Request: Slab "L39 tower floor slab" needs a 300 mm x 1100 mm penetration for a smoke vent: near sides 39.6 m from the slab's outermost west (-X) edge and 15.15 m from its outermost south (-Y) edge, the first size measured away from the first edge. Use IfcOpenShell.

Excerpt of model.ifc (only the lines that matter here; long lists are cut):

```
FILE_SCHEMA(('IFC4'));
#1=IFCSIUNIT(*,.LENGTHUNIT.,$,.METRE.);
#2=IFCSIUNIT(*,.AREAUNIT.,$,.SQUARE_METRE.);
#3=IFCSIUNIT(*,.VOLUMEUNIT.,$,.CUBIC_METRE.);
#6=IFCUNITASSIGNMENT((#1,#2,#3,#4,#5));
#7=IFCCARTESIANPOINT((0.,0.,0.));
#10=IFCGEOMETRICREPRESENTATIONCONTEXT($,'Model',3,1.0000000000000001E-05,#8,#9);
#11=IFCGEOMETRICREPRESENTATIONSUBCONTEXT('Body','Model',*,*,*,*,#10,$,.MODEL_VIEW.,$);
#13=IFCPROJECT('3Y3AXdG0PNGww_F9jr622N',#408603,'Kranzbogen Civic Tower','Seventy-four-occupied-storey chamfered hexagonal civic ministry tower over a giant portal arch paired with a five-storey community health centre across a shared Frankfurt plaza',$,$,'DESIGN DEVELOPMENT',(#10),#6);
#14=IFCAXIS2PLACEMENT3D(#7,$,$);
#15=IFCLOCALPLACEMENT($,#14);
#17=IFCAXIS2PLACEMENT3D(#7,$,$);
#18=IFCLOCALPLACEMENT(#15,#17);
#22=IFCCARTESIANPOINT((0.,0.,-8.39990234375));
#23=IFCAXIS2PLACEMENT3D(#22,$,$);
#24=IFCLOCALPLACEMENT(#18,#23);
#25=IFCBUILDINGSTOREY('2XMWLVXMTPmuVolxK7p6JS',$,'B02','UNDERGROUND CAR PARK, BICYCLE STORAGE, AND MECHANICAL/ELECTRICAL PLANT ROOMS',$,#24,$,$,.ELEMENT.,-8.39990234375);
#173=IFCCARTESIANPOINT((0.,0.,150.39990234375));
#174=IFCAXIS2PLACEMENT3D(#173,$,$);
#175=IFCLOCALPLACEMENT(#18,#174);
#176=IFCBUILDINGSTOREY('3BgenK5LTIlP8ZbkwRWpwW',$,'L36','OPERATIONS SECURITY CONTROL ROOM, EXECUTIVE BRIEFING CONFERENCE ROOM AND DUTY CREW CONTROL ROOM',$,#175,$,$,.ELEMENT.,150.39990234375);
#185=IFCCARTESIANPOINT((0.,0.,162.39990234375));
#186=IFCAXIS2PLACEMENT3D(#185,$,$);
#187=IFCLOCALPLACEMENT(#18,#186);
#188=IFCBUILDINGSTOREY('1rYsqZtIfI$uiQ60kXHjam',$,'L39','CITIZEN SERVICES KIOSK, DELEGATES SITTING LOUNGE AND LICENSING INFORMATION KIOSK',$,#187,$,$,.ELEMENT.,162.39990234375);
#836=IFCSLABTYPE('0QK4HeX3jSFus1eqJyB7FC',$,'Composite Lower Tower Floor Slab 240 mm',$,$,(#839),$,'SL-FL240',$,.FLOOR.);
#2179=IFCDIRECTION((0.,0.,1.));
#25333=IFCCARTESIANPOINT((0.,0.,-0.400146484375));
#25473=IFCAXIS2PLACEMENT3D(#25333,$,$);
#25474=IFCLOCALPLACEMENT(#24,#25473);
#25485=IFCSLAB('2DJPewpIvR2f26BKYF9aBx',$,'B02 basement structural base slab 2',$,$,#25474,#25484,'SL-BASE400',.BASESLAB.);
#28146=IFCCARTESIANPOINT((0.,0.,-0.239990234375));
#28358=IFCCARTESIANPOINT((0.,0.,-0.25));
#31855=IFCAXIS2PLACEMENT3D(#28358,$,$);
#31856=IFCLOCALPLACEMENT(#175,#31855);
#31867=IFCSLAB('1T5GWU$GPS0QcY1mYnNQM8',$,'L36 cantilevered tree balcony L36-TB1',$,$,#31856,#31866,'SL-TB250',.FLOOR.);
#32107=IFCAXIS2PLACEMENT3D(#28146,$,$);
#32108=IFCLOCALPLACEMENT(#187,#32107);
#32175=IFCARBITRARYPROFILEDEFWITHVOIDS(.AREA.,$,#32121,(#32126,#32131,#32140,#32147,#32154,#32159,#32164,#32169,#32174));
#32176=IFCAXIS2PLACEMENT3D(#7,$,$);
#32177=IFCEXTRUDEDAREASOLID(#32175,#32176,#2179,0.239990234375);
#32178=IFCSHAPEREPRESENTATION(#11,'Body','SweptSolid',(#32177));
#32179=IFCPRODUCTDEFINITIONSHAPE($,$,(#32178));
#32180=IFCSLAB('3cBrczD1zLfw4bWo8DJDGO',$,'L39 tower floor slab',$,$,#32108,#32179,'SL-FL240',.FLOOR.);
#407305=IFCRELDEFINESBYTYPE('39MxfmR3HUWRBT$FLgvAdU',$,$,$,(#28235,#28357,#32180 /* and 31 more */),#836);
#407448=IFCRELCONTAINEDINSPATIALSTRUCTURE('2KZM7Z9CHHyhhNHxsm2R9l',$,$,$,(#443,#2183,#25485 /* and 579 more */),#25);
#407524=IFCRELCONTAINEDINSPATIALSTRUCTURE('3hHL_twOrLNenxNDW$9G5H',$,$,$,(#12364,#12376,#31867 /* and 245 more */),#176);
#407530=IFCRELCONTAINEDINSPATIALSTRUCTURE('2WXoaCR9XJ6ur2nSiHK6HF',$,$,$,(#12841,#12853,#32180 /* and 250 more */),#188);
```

```python
import numpy as np
import ifcopenshell
import ifcopenshell.api.feature
import ifcopenshell.api.geometry
import ifcopenshell.api.root
import ifcopenshell.geom
import ifcopenshell.util.placement
import ifcopenshell.util.representation
import ifcopenshell.util.shape
import ifcopenshell.util.unit

model = ifcopenshell.open("model.ifc")
unit_scale = ifcopenshell.util.unit.calculate_unit_scale(model)
settings = ifcopenshell.geom.settings()


def volume(element):
    """Net volume in cubic metres, openings subtracted."""
    shape = ifcopenshell.geom.create_shape(settings, element)
    return ifcopenshell.util.shape.get_volume(shape.geometry)


slab = model.by_id(32180)
before = volume(slab)

# Extent in the slab's own axes, in metres. The edges named are its -X and -Y sides.
slab_shape = ifcopenshell.geom.create_shape(settings, slab)
vertices = ifcopenshell.util.shape.get_vertices(slab_shape.geometry)
x_min, y_min, bottom = vertices.min(axis=0)
top = vertices[:, 2].max()

opening = ifcopenshell.api.root.create_entity(model, ifc_class="IfcOpeningElement", name="Smoke vent opening", predefined_type="OPENING")
context = ifcopenshell.util.representation.get_context(model, "Model", "Body", "MODEL_VIEW")
width, depth = 0.3, 1.1
outline = [(0.0, 0.0), (width, 0.0), (width, depth), (0.0, depth), (0.0, 0.0)]
# Overshoot both faces by 50 mm so the cut is clean.
shape = ifcopenshell.api.geometry.add_slab_representation(
    model, context=context, depth=top - bottom + 0.1, polyline=outline
)
ifcopenshell.api.geometry.assign_representation(model, product=opening, representation=shape)

matrix = ifcopenshell.util.placement.get_local_placement(slab.ObjectPlacement)
matrix[:, 3] = matrix @ np.append(np.array([x_min + 39.6, y_min + 15.15, bottom - 0.05]) / unit_scale, 1.0)
ifcopenshell.api.geometry.edit_object_placement(model, product=opening, matrix=matrix, is_si=False)
ifcopenshell.api.feature.add_feature(model, feature=opening, element=slab)

after = volume(slab)

print(f"slab volume {before:.3f} -> {after:.3f} m3")

model.write("model_edited.ifc")
```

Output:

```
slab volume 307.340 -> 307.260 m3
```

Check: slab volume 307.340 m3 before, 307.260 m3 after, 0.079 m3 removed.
